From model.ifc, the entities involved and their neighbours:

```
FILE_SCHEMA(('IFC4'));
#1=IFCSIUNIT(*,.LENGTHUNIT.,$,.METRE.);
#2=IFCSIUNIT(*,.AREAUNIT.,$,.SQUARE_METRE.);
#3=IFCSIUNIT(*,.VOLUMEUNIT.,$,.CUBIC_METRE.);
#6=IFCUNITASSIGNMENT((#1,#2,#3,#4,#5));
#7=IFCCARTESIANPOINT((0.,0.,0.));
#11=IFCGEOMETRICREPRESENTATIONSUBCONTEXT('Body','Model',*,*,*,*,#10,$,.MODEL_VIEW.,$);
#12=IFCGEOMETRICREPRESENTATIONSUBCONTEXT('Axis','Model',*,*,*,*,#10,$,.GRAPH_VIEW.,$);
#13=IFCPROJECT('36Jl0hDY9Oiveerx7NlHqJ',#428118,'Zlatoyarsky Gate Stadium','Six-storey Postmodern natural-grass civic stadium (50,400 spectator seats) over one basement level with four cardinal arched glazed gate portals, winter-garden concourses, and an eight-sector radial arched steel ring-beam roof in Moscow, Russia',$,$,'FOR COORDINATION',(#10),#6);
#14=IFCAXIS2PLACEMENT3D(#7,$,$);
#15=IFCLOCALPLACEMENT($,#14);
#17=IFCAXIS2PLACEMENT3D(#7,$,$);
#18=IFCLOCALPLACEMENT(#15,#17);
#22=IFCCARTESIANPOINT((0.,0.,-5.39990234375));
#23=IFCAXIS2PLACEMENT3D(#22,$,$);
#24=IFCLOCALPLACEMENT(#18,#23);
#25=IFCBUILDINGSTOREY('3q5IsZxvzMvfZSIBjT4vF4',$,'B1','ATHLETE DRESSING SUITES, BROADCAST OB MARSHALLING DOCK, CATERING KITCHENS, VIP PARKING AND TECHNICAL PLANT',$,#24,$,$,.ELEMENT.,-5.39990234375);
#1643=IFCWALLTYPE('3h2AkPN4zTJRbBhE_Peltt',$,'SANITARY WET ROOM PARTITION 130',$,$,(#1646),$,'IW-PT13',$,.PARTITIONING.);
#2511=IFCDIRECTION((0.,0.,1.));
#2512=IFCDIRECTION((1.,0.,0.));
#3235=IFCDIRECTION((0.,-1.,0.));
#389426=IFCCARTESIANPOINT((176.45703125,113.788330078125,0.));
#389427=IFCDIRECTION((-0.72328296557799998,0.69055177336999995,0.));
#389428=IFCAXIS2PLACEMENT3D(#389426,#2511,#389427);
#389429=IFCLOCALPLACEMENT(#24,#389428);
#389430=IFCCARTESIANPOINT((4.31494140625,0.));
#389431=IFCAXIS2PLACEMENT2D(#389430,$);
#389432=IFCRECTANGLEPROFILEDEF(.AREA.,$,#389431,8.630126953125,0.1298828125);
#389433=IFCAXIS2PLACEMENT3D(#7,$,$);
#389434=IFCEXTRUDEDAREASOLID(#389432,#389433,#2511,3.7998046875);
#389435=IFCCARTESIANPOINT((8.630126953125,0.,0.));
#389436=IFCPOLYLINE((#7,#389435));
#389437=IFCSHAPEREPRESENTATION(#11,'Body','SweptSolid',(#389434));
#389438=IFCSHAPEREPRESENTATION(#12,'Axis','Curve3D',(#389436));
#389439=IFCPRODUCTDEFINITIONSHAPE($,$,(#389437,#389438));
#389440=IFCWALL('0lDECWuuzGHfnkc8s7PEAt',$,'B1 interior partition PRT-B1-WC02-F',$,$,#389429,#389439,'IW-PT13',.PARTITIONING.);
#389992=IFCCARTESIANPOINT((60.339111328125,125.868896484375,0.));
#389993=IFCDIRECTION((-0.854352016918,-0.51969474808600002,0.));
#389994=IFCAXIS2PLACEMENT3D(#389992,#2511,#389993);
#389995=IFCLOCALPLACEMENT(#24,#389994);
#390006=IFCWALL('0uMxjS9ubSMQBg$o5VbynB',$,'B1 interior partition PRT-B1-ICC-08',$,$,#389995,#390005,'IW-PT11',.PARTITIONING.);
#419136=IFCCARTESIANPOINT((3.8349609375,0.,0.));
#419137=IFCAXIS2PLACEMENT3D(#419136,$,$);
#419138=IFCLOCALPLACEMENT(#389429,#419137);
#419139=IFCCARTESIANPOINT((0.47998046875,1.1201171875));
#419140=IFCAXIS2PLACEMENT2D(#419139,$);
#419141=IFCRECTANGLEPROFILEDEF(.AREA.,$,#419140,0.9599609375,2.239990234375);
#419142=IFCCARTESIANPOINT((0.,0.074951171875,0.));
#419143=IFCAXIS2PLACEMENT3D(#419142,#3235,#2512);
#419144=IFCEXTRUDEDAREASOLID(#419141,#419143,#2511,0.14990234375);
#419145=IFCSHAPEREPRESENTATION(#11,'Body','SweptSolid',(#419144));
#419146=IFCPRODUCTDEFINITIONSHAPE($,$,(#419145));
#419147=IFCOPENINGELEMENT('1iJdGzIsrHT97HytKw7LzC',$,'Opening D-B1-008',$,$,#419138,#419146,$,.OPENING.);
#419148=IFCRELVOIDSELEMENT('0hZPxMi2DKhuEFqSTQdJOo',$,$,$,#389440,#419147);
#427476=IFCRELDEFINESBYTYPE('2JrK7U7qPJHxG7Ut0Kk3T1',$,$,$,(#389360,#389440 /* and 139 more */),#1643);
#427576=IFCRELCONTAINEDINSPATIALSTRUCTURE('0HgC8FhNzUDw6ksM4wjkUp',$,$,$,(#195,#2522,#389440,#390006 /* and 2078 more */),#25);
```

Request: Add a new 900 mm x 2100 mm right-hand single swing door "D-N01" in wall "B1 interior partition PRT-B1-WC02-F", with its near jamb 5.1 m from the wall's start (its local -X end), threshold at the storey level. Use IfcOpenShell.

```python
import numpy as np
import ifcopenshell
import ifcopenshell.api.feature
import ifcopenshell.api.geometry
import ifcopenshell.api.root
import ifcopenshell.api.spatial
import ifcopenshell.geom
import ifcopenshell.util.element
import ifcopenshell.util.placement
import ifcopenshell.util.representation
import ifcopenshell.util.shape
import ifcopenshell.util.unit

model = ifcopenshell.open("model.ifc")
unit_scale = ifcopenshell.util.unit.calculate_unit_scale(model)
settings = ifcopenshell.geom.settings()


def volume(element):
    """Net volume in cubic metres, openings subtracted."""
    shape = ifcopenshell.geom.create_shape(settings, element)
    return ifcopenshell.util.shape.get_volume(shape.geometry)


wall = model.by_guid("0lDECWuuzGHfnkc8s7PEAt")
storey = ifcopenshell.util.element.get_container(wall, ifc_class="IfcBuildingStorey")
context = ifcopenshell.util.representation.get_context(model, "Model", "Body", "MODEL_VIEW")
before = volume(wall)

width, height, from_end, sill = 0.9, 2.1, 5.1, 0.0  # metres

# The wall runs along its own X axis, and the end named is its -X end.
wall_shape = ifcopenshell.geom.create_shape(settings, wall)
x, y, z = ifcopenshell.util.shape.get_vertices(wall_shape.geometry).T
start = x.min() + from_end
face, thickness = float(y.min()), float(y.max() - y.min())
wall_matrix = ifcopenshell.util.placement.get_local_placement(wall.ObjectPlacement)
level = ifcopenshell.util.placement.get_local_placement(storey.ObjectPlacement)[2, 3]


def in_wall(x, y):
    """Placement at x, y metres in the wall's axes, at sill height."""
    matrix = wall_matrix.copy()
    matrix[:, 3] = wall_matrix @ np.array([x / unit_scale, y / unit_scale, 0.0, 1.0])
    matrix[2, 3] = level + sill / unit_scale
    return matrix


# Opening: a box that overshoots both wall faces by 50 mm.
opening = ifcopenshell.api.root.create_entity(model, ifc_class="IfcOpeningElement", predefined_type="OPENING")
box = ifcopenshell.api.geometry.add_wall_representation(
    model, context=context, length=width, height=height, thickness=thickness + 0.1
)
ifcopenshell.api.geometry.assign_representation(model, product=opening, representation=box)
ifcopenshell.api.geometry.edit_object_placement(model, product=opening, matrix=in_wall(start, face - 0.05), is_si=False)
ifcopenshell.api.feature.add_feature(model, feature=opening, element=wall)

door = ifcopenshell.api.root.create_entity(model, ifc_class="IfcDoor", name="D-N01", predefined_type="DOOR")
door.OverallWidth, door.OverallHeight = width / unit_scale, height / unit_scale
door.OperationType = "SINGLE_SWING_RIGHT"
body = ifcopenshell.api.geometry.add_door_representation(
    model,
    context=context,
    overall_width=door.OverallWidth,
    overall_height=door.OverallHeight,
    operation_type="SINGLE_SWING_RIGHT",
    lining_properties={"LiningDepth": thickness / unit_scale, "ThresholdDepth": thickness / unit_scale},
)
ifcopenshell.api.geometry.assign_representation(model, product=door, representation=body)
ifcopenshell.api.spatial.assign_container(model, products=[door], relating_structure=storey)
ifcopenshell.api.feature.add_filling(model, opening=opening, element=door)

# The lining spans the wall, so the door starts at the wall face.
ifcopenshell.api.geometry.edit_object_placement(model, product=door, matrix=in_wall(start, face), is_si=False)

after = volume(wall)

print(f"wall volume {before:.3f} -> {after:.3f} m3")

model.write("model_v2.ifc")
```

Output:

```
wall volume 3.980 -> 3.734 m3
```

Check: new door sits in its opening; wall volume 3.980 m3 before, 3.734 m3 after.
